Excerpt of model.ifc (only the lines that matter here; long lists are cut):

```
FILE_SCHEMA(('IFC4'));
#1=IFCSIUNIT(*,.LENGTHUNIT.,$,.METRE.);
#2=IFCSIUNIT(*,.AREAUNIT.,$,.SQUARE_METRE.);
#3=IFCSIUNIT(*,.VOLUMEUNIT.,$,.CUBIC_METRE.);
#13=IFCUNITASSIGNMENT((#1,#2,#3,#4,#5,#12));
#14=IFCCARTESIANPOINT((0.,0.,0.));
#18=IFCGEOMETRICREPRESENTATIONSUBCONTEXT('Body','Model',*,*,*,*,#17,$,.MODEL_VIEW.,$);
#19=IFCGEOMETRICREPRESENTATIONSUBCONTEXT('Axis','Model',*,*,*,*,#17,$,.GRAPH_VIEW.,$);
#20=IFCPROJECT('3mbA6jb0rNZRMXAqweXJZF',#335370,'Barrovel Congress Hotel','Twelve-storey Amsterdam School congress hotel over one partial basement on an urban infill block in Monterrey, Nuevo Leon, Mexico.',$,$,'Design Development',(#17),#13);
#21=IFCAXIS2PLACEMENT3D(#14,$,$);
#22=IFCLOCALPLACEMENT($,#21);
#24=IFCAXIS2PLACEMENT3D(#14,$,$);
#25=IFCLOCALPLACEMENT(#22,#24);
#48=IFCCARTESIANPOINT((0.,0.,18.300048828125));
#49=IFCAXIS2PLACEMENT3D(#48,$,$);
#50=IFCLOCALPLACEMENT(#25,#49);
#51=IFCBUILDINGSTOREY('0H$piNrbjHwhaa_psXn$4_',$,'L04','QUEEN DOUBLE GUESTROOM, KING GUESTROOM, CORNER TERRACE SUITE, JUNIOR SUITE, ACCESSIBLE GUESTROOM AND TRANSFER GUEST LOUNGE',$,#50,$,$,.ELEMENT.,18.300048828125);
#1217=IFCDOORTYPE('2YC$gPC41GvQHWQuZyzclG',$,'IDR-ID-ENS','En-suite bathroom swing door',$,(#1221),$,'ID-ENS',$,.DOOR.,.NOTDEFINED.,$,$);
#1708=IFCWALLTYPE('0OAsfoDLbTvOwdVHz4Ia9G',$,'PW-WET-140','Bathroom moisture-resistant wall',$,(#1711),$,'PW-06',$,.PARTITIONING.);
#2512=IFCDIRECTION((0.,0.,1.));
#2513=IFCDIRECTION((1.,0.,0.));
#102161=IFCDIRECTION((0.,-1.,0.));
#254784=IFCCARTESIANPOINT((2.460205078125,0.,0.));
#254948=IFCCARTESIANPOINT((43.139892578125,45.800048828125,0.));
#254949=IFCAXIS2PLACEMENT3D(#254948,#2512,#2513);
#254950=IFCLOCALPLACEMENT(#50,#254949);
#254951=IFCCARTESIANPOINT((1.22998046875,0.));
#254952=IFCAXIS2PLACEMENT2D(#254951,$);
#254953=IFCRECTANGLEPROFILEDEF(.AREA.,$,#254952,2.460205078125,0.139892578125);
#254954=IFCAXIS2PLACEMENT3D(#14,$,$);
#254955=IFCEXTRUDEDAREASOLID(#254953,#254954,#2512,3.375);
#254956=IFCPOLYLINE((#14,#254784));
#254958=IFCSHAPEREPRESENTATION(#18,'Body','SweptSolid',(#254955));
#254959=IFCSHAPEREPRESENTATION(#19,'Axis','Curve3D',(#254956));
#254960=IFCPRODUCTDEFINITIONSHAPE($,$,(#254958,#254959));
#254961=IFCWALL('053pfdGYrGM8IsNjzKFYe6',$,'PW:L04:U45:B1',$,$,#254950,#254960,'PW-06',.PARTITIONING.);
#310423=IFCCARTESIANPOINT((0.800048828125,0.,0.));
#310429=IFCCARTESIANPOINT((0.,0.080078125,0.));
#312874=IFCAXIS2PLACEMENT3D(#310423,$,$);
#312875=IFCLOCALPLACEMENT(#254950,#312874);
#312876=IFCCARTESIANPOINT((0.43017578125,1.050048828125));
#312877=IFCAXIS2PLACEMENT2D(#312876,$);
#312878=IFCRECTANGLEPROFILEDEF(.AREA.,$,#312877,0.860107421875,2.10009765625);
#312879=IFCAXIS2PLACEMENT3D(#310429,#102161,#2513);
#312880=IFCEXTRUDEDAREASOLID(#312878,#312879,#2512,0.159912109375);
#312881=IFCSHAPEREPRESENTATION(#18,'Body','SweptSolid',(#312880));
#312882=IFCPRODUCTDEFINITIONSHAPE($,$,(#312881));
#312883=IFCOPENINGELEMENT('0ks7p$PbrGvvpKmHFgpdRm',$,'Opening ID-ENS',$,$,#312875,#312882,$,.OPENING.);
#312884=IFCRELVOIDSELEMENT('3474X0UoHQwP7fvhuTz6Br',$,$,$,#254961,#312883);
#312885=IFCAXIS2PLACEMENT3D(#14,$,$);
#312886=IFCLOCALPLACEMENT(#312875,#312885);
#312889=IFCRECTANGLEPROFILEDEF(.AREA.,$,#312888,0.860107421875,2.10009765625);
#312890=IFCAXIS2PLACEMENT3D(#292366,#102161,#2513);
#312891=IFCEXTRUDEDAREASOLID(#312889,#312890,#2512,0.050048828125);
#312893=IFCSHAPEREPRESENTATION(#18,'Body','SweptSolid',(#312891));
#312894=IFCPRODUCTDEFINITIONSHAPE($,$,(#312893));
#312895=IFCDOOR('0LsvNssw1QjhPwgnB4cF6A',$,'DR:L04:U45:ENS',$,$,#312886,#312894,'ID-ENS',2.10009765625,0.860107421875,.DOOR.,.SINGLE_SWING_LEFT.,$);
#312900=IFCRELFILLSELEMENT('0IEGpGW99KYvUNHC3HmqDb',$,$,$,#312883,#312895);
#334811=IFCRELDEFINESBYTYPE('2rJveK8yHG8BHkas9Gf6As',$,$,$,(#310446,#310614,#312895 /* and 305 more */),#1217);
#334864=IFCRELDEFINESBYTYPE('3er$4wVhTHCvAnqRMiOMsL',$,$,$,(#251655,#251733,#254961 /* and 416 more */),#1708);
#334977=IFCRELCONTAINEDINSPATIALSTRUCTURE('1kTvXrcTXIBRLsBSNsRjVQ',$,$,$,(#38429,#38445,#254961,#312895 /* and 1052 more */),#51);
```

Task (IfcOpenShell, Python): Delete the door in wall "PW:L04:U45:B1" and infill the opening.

```python
import ifcopenshell
import ifcopenshell.api.feature
import ifcopenshell.api.root
import ifcopenshell.geom
import ifcopenshell.util.shape

model = ifcopenshell.open("model.ifc")
settings = ifcopenshell.geom.settings()


def volume(element):
    """Net volume in cubic metres, openings subtracted."""
    shape = ifcopenshell.geom.create_shape(settings, element)
    return ifcopenshell.util.shape.get_volume(shape.geometry)


door = model.by_id(312895)
opening = door.FillsVoids[0].RelatingOpeningElement
wall = opening.VoidsElements[0].RelatingBuildingElement
before = volume(wall)

ifcopenshell.api.root.remove_product(model, product=door)
ifcopenshell.api.feature.remove_feature(model, feature=opening)

after = volume(wall)

print(f"wall volume {before:.3f} -> {after:.3f} m3")

model.write("model_edited.ifc")
```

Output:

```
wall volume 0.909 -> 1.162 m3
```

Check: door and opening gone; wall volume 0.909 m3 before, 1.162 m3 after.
